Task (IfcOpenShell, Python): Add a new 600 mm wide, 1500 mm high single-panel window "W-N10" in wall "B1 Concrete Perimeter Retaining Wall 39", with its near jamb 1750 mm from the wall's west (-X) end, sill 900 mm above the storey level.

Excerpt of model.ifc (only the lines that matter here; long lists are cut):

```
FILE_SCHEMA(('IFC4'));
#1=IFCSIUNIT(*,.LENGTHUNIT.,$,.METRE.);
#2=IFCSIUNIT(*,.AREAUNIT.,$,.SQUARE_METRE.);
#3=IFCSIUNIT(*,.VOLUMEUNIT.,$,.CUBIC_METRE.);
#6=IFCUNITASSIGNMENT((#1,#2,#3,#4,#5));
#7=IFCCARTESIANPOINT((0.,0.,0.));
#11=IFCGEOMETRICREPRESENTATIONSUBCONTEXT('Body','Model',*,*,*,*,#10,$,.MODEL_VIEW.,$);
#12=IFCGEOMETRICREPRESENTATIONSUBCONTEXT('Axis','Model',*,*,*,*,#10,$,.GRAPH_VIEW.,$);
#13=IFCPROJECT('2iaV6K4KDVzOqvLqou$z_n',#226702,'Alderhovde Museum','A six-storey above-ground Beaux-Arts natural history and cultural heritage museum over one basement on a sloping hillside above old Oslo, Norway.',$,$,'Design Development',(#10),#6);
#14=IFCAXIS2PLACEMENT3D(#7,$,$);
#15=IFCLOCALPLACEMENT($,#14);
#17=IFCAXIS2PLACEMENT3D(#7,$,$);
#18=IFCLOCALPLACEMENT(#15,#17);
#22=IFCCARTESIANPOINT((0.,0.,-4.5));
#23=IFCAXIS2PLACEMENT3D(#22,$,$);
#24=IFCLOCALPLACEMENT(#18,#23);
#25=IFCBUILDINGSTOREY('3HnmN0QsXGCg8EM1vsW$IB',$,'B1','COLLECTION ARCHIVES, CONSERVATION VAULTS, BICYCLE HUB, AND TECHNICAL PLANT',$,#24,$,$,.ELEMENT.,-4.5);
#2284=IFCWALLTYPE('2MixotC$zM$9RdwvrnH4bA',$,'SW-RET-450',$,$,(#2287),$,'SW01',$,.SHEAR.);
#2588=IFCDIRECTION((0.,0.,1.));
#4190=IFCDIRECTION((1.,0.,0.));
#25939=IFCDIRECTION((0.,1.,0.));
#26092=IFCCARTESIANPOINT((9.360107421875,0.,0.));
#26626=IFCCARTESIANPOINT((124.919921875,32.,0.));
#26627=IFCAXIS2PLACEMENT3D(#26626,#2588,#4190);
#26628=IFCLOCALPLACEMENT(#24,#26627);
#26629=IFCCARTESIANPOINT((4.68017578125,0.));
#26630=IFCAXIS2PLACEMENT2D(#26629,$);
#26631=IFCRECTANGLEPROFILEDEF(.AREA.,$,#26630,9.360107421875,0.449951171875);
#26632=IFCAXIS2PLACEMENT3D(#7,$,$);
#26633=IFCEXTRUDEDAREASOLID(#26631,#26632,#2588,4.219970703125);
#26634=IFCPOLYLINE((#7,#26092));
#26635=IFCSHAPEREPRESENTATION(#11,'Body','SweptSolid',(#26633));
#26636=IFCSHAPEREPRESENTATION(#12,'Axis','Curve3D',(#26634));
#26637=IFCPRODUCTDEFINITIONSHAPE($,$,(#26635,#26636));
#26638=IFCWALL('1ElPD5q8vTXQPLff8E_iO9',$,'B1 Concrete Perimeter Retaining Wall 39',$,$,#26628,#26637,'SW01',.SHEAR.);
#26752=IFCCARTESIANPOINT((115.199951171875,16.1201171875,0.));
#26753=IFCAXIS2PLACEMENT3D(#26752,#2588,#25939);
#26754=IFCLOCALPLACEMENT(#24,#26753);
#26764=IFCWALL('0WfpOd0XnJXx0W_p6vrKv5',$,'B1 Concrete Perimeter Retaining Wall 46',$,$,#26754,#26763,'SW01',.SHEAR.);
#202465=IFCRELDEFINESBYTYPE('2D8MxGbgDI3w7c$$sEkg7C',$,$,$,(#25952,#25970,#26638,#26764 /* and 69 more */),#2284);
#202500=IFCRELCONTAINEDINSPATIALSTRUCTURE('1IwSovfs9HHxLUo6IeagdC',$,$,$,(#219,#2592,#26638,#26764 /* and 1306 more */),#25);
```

```python
import numpy as np
import ifcopenshell
import ifcopenshell.api.feature
import ifcopenshell.api.geometry
import ifcopenshell.api.root
import ifcopenshell.api.spatial
import ifcopenshell.geom
import ifcopenshell.util.element
import ifcopenshell.util.placement
import ifcopenshell.util.representation
import ifcopenshell.util.shape
import ifcopenshell.util.unit

model = ifcopenshell.open("model.ifc")
unit_scale = ifcopenshell.util.unit.calculate_unit_scale(model)
settings = ifcopenshell.geom.settings()


def volume(element):
    """Net volume in cubic metres, openings subtracted."""
    shape = ifcopenshell.geom.create_shape(settings, element)
    return ifcopenshell.util.shape.get_volume(shape.geometry)


wall = model.by_id(26638)
storey = ifcopenshell.util.element.get_container(wall, ifc_class="IfcBuildingStorey")
context = ifcopenshell.util.representation.get_context(model, "Model", "Body", "MODEL_VIEW")
before = volume(wall)

width, height, from_end, sill = 0.6, 1.5, 1.75, 0.9  # metres

# The wall runs along its own X axis, and the end named is its -X end.
wall_shape = ifcopenshell.geom.create_shape(settings, wall)
x, y, z = ifcopenshell.util.shape.get_vertices(wall_shape.geometry).T
start = x.min() + from_end
face, thickness = float(y.min()), float(y.max() - y.min())
wall_matrix = ifcopenshell.util.placement.get_local_placement(wall.ObjectPlacement)
level = ifcopenshell.util.placement.get_local_placement(storey.ObjectPlacement)[2, 3]


def in_wall(x, y):
    """Placement at x, y metres in the wall's axes, at sill height."""
    matrix = wall_matrix.copy()
    matrix[:, 3] = wall_matrix @ np.array([x / unit_scale, y / unit_scale, 0.0, 1.0])
    matrix[2, 3] = level + sill / unit_scale
    return matrix


# Opening: a box that overshoots both wall faces by 50 mm.
opening = ifcopenshell.api.root.create_entity(model, ifc_class="IfcOpeningElement", predefined_type="OPENING")
box = ifcopenshell.api.geometry.add_wall_representation(
    model, context=context, length=width, height=height, thickness=thickness + 0.1
)
ifcopenshell.api.geometry.assign_representation(model, product=opening, representation=box)
ifcopenshell.api.geometry.edit_object_placement(model, product=opening, matrix=in_wall(start, face - 0.05), is_si=False)
ifcopenshell.api.feature.add_feature(model, feature=opening, element=wall)

window = ifcopenshell.api.root.create_entity(model, ifc_class="IfcWindow", name="W-N10", predefined_type="WINDOW")
window.OverallWidth, window.OverallHeight = width / unit_scale, height / unit_scale
window.PartitioningType = "SINGLE_PANEL"
body = ifcopenshell.api.geometry.add_window_representation(
    model,
    context=context,
    overall_width=window.OverallWidth,
    overall_height=window.OverallHeight,
    partition_type="SINGLE_PANEL",
)
ifcopenshell.api.geometry.assign_representation(model, product=window, representation=body)
ifcopenshell.api.spatial.assign_container(model, products=[window], relating_structure=storey)
ifcopenshell.api.feature.add_filling(model, opening=opening, element=window)

# Centre the window in the wall's thickness.
ifcopenshell.api.geometry.edit_object_placement(model, product=window, matrix=in_wall(start, face), is_si=False)
window_shape = ifcopenshell.geom.create_shape(settings, window)
depth = ifcopenshell.util.shape.get_vertices(window_shape.geometry)[:, 1]
offset = face + thickness / 2 - (depth.min() + depth.max()) / 2
ifcopenshell.api.geometry.edit_object_placement(model, product=window, matrix=in_wall(start, offset), is_si=False)

after = volume(wall)

print(f"wall volume {before:.3f} -> {after:.3f} m3")

model.write("model-out.ifc")
```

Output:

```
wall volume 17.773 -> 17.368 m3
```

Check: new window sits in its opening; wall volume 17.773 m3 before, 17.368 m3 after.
